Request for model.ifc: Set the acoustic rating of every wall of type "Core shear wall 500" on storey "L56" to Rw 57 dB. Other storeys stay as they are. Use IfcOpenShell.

First a look at what the model holds.

```python
import ifcopenshell
import ifcopenshell.util.element

model = ifcopenshell.open("model.ifc")
print(model.schema)
storey = next(s for s in model.by_type("IfcBuildingStorey") if s.Name == "L56")
walls = [e for e in ifcopenshell.util.element.get_decomposition(storey) if e.is_a("IfcWall")]
seen = {}
for e in walls:
    element_type = ifcopenshell.util.element.get_type(e)
    key = (element_type.Name if element_type != e and element_type else None, ifcopenshell.util.element.get_pset(e, "Pset_WallCommon", "AcousticRating"))
    seen[key] = seen.get(key, 0) + 1
for (name, value), count in sorted(seen.items(), key=str):
    print(count, "x", name, "|", value)
```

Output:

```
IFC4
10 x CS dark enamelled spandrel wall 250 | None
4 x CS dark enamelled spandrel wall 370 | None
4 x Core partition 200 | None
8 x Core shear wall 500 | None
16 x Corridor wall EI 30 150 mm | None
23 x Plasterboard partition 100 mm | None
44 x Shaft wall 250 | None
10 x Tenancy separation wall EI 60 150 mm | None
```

```python
import ifcopenshell
import ifcopenshell.api.pset
import ifcopenshell.util.element

model = ifcopenshell.open("model.ifc")

storey = next(s for s in model.by_type("IfcBuildingStorey") if s.Name == "L56")
walls = [e for e in ifcopenshell.util.element.get_decomposition(storey) if e.is_a("IfcWall")]

count = 0
for e in walls:
    element_type = ifcopenshell.util.element.get_type(e)
    if element_type in (None, e) or element_type.Name != "Core shear wall 500":
        continue
    found = ifcopenshell.util.element.get_pset(e, "Pset_WallCommon", should_inherit=False)
    if found:
        pset = model.by_id(found["id"])
        if len(ifcopenshell.util.element.get_elements_by_pset(pset)) > 1:
            pset = ifcopenshell.api.pset.unshare_pset(model, products=[e], pset=pset)[0]
    else:
        pset = ifcopenshell.api.pset.add_pset(model, product=e, name="Pset_WallCommon")
    ifcopenshell.api.pset.edit_pset(model, pset=pset, properties={"AcousticRating": "Rw 57 dB"})
    count += 1

print(count, "walls updated")

model.write("model_edited.ifc")
```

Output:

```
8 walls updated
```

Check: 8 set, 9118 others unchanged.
